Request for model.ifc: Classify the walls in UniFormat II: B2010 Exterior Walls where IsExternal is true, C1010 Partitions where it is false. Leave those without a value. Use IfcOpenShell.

First a look at what the model holds.

```python
import ifcopenshell
import ifcopenshell.util.element

model = ifcopenshell.open("model.ifc")
print(model.schema)
print("classifications:", [c.Name for c in model.by_type("IfcClassification")])
values = [ifcopenshell.util.element.get_pset(e, "Pset_WallCommon", "IsExternal") for e in model.by_type("IfcWall")]
for value in (True, False, None):
    print("IsExternal", value, values.count(value))
```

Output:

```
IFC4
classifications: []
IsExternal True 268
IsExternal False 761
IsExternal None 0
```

```python
import ifcopenshell
import ifcopenshell.api.classification
import ifcopenshell.util.element

model = ifcopenshell.open("model.ifc")

system = ifcopenshell.api.classification.add_classification(model, classification="UniFormat II")

walls = model.by_type("IfcWall")
external = {e: ifcopenshell.util.element.get_pset(e, "Pset_WallCommon", "IsExternal") for e in walls}
for flag, code, name in ((True, "B2010", "Exterior Walls"), (False, "C1010", "Partitions")):
    products = [e for e in walls if external[e] is flag]
    ifcopenshell.api.classification.add_reference(
        model, products=products, classification=system, identification=code, name=name
    )
    print(code, len(products))

model.write("model_updated.ifc")
```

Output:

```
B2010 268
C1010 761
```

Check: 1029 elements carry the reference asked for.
